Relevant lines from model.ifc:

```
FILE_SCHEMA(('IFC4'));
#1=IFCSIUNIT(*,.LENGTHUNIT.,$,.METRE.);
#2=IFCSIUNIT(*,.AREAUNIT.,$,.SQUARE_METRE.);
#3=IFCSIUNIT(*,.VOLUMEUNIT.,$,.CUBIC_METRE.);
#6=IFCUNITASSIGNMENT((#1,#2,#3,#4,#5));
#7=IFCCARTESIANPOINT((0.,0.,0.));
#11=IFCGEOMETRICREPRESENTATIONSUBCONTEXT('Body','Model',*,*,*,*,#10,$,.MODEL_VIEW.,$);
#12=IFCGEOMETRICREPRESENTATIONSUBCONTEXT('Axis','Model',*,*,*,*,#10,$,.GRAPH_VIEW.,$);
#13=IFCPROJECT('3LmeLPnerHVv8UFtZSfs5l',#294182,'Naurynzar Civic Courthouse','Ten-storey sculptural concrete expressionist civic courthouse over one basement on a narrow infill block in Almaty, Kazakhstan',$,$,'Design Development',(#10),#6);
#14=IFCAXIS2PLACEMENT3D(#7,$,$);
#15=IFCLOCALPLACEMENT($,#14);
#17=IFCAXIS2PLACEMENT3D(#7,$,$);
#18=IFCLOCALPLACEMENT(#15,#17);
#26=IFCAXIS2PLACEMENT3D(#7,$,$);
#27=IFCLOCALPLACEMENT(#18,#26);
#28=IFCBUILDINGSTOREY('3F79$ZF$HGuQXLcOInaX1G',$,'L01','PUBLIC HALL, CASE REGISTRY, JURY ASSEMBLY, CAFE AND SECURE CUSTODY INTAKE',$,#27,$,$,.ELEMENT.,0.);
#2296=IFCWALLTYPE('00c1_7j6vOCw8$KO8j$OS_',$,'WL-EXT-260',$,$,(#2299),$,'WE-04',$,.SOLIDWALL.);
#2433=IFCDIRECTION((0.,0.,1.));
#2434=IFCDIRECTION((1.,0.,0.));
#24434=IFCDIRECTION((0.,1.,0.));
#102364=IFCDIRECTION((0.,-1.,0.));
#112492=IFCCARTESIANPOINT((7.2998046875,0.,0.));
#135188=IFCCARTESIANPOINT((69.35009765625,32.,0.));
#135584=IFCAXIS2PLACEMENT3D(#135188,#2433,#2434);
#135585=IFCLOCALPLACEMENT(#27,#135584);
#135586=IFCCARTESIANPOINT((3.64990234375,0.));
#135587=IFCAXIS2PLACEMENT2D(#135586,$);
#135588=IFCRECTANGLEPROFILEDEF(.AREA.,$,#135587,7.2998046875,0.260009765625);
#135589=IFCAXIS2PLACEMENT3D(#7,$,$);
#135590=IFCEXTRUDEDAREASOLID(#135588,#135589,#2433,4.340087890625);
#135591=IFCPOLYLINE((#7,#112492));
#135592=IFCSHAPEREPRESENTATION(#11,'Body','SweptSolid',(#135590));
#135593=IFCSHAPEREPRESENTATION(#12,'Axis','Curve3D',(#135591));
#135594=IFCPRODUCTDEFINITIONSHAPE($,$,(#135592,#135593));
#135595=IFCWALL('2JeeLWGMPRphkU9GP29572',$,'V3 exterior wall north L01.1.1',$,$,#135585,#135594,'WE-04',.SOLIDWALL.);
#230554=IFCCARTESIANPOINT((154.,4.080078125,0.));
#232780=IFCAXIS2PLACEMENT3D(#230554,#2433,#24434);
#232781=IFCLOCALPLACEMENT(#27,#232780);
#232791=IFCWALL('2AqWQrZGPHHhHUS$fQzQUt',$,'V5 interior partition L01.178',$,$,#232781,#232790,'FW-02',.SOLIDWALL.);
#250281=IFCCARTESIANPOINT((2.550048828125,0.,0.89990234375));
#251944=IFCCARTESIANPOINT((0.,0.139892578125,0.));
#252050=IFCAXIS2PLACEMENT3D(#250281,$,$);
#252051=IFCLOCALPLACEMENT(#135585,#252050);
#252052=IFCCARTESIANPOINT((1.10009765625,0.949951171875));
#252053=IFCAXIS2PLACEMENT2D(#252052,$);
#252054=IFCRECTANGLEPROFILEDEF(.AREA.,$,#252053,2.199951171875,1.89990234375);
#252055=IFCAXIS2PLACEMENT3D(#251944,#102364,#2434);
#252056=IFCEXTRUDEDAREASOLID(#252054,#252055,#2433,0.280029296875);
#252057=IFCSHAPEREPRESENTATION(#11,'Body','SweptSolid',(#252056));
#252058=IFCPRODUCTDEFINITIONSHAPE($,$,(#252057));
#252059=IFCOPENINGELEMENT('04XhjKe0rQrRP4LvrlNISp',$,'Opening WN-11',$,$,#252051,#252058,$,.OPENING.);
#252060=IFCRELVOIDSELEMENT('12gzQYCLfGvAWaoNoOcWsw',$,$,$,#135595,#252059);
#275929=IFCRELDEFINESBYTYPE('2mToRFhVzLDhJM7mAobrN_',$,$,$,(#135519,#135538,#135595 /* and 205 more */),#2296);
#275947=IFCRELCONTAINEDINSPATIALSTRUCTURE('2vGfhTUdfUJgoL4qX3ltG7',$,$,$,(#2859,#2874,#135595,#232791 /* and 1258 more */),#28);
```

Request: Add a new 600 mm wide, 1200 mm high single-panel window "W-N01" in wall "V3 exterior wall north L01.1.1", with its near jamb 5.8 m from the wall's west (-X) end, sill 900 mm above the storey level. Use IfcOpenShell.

```python
import numpy as np
import ifcopenshell
import ifcopenshell.api.feature
import ifcopenshell.api.geometry
import ifcopenshell.api.root
import ifcopenshell.api.spatial
import ifcopenshell.geom
import ifcopenshell.util.element
import ifcopenshell.util.placement
import ifcopenshell.util.representation
import ifcopenshell.util.shape
import ifcopenshell.util.unit

model = ifcopenshell.open("model.ifc")
unit_scale = ifcopenshell.util.unit.calculate_unit_scale(model)
settings = ifcopenshell.geom.settings()


def volume(element):
    """Net volume in cubic metres, openings subtracted."""
    shape = ifcopenshell.geom.create_shape(settings, element)
    return ifcopenshell.util.shape.get_volume(shape.geometry)


wall = model.by_guid("2JeeLWGMPRphkU9GP29572")
storey = ifcopenshell.util.element.get_container(wall, ifc_class="IfcBuildingStorey")
context = ifcopenshell.util.representation.get_context(model, "Model", "Body", "MODEL_VIEW")
before = volume(wall)

width, height, from_end, sill = 0.6, 1.2, 5.8, 0.9  # metres

# The wall runs along its own X axis, and the end named is its -X end.
wall_shape = ifcopenshell.geom.create_shape(settings, wall)
x, y, z = ifcopenshell.util.shape.get_vertices(wall_shape.geometry).T
start = x.min() + from_end
face, thickness = float(y.min()), float(y.max() - y.min())
wall_matrix = ifcopenshell.util.placement.get_local_placement(wall.ObjectPlacement)
level = ifcopenshell.util.placement.get_local_placement(storey.ObjectPlacement)[2, 3]


def in_wall(x, y):
    """Placement at x, y metres in the wall's axes, at sill height."""
    matrix = wall_matrix.copy()
    matrix[:, 3] = wall_matrix @ np.array([x / unit_scale, y / unit_scale, 0.0, 1.0])
    matrix[2, 3] = level + sill / unit_scale
    return matrix


# Opening: a box that overshoots both wall faces by 50 mm.
opening = ifcopenshell.api.root.create_entity(model, ifc_class="IfcOpeningElement", predefined_type="OPENING")
box = ifcopenshell.api.geometry.add_wall_representation(
    model, context=context, length=width, height=height, thickness=thickness + 0.1
)
ifcopenshell.api.geometry.assign_representation(model, product=opening, representation=box)
ifcopenshell.api.geometry.edit_object_placement(model, product=opening, matrix=in_wall(start, face - 0.05), is_si=False)
ifcopenshell.api.feature.add_feature(model, feature=opening, element=wall)

window = ifcopenshell.api.root.create_entity(model, ifc_class="IfcWindow", name="W-N01", predefined_type="WINDOW")
window.OverallWidth, window.OverallHeight = width / unit_scale, height / unit_scale
window.PartitioningType = "SINGLE_PANEL"
body = ifcopenshell.api.geometry.add_window_representation(
    model,
    context=context,
    overall_width=window.OverallWidth,
    overall_height=window.OverallHeight,
    partition_type="SINGLE_PANEL",
)
ifcopenshell.api.geometry.assign_representation(model, product=window, representation=body)
ifcopenshell.api.spatial.assign_container(model, products=[window], relating_structure=storey)
ifcopenshell.api.feature.add_filling(model, opening=opening, element=window)

# Centre the window in the wall's thickness.
ifcopenshell.api.geometry.edit_object_placement(model, product=window, matrix=in_wall(start, face), is_si=False)
window_shape = ifcopenshell.geom.create_shape(settings, window)
depth = ifcopenshell.util.shape.get_vertices(window_shape.geometry)[:, 1]
offset = face + thickness / 2 - (depth.min() + depth.max()) / 2
ifcopenshell.api.geometry.edit_object_placement(model, product=window, matrix=in_wall(start, offset), is_si=False)

after = volume(wall)

print(f"wall volume {before:.3f} -> {after:.3f} m3")

model.write("model_edited.ifc")
```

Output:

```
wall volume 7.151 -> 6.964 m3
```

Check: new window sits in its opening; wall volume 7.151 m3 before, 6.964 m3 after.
